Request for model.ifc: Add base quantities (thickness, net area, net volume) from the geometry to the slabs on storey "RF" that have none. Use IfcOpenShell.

First a look at what the model holds.

```python
import ifcopenshell
import ifcopenshell.util.element
import ifcopenshell.util.unit

model = ifcopenshell.open("model.ifc")
print(model.schema)
for unit_type in ("LENGTHUNIT", "AREAUNIT", "VOLUMEUNIT"):
    print(unit_type, ifcopenshell.util.unit.calculate_unit_scale(model, unit_type))
storey = next(s for s in model.by_type("IfcBuildingStorey") if s.Name == "RF")
slabs = [e for e in ifcopenshell.util.element.get_decomposition(storey) if e.is_a("IfcSlab")]
for e in sorted(slabs, key=lambda e: e.id()):
    print(e.id(), e.is_a(), e.Name, list(ifcopenshell.util.element.get_psets(e, qtos_only=True)), sep=" | ")
```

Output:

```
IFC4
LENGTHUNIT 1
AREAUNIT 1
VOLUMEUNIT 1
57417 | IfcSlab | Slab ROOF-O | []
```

```python
import ifcopenshell
import ifcopenshell.api.pset
import ifcopenshell.geom
import ifcopenshell.util.element
import ifcopenshell.util.shape
import ifcopenshell.util.unit

model = ifcopenshell.open("model.ifc")
unit_scale = ifcopenshell.util.unit.calculate_unit_scale(model)
area_scale = ifcopenshell.util.unit.calculate_unit_scale(model, "AREAUNIT")
volume_scale = ifcopenshell.util.unit.calculate_unit_scale(model, "VOLUMEUNIT")
settings = ifcopenshell.geom.settings()

storey = next(s for s in model.by_type("IfcBuildingStorey") if s.Name == "RF")
slabs = [e for e in ifcopenshell.util.element.get_decomposition(storey) if e.is_a("IfcSlab")]

for e in sorted(slabs, key=lambda e: e.id()):
    if ifcopenshell.util.element.get_psets(e, qtos_only=True, should_inherit=False):
        continue
    # Geometry comes back in metres, in the element's own axes.
    shape = ifcopenshell.geom.create_shape(settings, e)
    values = {
        "Width": ifcopenshell.util.shape.get_z(shape.geometry) / unit_scale,
        "NetArea": ifcopenshell.util.shape.get_footprint_area(shape.geometry) / area_scale,
        "NetVolume": ifcopenshell.util.shape.get_volume(shape.geometry) / volume_scale,
    }
    qto = ifcopenshell.api.pset.add_qto(model, product=e, name="Qto_SlabBaseQuantities")
    ifcopenshell.api.pset.edit_qto(model, qto=qto, properties=values)
    print(e.id(), {k: round(v, 3) for k, v in values.items()})

model.write("model-out.ifc")
```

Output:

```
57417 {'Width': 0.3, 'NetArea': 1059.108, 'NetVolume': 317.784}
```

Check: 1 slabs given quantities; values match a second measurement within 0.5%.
